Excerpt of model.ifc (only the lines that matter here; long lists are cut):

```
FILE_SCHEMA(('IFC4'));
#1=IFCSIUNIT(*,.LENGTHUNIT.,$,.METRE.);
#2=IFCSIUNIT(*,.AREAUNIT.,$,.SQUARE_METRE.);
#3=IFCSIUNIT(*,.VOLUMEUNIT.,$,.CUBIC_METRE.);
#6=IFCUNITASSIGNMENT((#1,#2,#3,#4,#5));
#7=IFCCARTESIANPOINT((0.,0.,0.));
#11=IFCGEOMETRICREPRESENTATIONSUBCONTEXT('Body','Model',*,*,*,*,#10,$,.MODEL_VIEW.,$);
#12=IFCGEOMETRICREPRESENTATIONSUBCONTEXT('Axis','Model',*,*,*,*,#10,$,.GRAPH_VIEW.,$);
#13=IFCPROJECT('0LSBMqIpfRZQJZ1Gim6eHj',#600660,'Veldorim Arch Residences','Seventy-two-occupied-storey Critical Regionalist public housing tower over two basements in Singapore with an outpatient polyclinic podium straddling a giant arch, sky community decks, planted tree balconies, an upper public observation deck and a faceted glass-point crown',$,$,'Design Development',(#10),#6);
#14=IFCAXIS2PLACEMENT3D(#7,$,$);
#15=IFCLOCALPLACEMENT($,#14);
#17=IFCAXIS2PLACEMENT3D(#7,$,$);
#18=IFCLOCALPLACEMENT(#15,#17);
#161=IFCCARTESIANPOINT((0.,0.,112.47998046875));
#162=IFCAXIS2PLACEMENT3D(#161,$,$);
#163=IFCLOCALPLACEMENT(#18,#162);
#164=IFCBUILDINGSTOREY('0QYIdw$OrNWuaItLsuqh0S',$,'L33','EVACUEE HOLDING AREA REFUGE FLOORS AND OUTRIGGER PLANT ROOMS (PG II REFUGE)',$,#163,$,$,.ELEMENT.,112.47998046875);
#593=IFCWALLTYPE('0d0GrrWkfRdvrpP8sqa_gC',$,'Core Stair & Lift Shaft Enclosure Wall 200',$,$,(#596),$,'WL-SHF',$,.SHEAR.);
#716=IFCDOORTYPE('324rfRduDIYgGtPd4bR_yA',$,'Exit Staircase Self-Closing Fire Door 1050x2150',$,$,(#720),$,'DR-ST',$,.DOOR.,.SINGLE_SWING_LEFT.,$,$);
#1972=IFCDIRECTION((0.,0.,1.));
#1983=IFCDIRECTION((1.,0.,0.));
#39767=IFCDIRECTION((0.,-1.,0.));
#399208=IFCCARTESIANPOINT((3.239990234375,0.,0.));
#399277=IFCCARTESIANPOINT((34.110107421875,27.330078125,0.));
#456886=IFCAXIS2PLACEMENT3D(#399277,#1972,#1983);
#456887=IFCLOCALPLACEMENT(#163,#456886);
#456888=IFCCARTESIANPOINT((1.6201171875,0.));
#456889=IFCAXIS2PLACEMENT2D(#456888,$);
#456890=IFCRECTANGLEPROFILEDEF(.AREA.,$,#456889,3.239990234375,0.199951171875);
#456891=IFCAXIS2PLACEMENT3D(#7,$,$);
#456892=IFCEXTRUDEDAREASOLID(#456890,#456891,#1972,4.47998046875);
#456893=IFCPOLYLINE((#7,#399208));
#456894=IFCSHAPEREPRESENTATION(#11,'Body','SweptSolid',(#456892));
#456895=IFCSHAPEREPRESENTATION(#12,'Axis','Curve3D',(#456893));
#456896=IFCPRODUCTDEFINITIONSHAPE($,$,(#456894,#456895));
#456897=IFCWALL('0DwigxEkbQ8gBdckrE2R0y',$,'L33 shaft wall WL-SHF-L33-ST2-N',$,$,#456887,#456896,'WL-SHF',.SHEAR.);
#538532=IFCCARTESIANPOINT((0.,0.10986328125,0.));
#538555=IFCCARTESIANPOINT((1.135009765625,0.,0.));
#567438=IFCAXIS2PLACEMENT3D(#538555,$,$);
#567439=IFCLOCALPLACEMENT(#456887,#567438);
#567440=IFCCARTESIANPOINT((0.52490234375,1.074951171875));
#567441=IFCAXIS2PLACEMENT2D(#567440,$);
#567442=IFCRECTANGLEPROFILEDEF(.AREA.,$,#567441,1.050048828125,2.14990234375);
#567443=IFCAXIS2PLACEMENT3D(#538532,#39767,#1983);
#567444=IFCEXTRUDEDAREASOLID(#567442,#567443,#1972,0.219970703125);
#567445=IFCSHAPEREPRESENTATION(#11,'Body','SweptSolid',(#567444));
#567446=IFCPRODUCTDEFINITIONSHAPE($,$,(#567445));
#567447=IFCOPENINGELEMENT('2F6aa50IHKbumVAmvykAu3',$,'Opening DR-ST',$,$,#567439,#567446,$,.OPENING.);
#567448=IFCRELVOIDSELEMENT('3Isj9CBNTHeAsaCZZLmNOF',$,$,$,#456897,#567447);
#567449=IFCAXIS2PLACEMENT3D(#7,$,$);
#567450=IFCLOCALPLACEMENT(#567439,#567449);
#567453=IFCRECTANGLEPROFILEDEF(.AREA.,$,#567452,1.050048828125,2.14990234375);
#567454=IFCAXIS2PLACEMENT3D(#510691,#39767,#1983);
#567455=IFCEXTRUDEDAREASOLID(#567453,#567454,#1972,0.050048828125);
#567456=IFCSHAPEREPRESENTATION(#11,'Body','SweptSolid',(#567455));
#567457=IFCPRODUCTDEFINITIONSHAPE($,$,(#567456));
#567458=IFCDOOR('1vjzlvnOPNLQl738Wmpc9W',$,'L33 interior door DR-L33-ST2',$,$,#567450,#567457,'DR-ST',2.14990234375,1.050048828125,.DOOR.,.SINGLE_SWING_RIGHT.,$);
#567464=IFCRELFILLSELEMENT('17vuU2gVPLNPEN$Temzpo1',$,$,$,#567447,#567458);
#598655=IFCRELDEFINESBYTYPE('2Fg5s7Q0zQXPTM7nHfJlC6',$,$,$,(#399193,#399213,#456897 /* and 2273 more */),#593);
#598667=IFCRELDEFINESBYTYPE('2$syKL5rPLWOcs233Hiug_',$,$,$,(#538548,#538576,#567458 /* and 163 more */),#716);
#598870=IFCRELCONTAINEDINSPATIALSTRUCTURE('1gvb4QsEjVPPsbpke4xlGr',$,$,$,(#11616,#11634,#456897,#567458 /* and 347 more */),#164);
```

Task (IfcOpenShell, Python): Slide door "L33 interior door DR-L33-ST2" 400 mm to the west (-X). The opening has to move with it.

```python
import ifcopenshell
import ifcopenshell.api.geometry
import ifcopenshell.util.placement

model = ifcopenshell.open("model.ifc")

door = model.by_guid("1vjzlvnOPNLQl738Wmpc9W")
opening = door.FillsVoids[0].RelatingOpeningElement
wall = opening.VoidsElements[0].RelatingBuildingElement

wall_matrix = ifcopenshell.util.placement.get_local_placement(wall.ObjectPlacement)
shift = wall_matrix[:3, 0] * -0.4
before = ifcopenshell.util.placement.get_local_placement(door.ObjectPlacement)[:3, 3].copy()

# The door is placed relative to its opening, so it follows when the opening moves.
matrix = ifcopenshell.util.placement.get_local_placement(opening.ObjectPlacement)
matrix[:3, 3] += shift
ifcopenshell.api.geometry.edit_object_placement(
    model, product=opening, matrix=matrix, is_si=False, should_transform_children=True
)

after = ifcopenshell.util.placement.get_local_placement(door.ObjectPlacement)[:3, 3]
print("door moved by", (after - before).round(3) + 0.0)

model.write("model-out.ifc")
```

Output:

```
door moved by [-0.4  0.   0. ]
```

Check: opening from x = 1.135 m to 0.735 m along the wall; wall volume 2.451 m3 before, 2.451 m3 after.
